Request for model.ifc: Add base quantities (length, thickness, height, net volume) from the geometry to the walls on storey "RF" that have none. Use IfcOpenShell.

First a look at what the model holds.

```python
import ifcopenshell
import ifcopenshell.util.element
import ifcopenshell.util.unit

model = ifcopenshell.open("model.ifc")
print(model.schema)
for unit_type in ("LENGTHUNIT", "AREAUNIT", "VOLUMEUNIT"):
    print(unit_type, ifcopenshell.util.unit.calculate_unit_scale(model, unit_type))
storey = next(s for s in model.by_type("IfcBuildingStorey") if s.Name == "RF")
walls = [e for e in ifcopenshell.util.element.get_decomposition(storey) if e.is_a("IfcWall")]
for e in sorted(walls, key=lambda e: e.id()):
    print(e.id(), e.is_a(), e.Name, list(ifcopenshell.util.element.get_psets(e, qtos_only=True)), sep=" | ")
```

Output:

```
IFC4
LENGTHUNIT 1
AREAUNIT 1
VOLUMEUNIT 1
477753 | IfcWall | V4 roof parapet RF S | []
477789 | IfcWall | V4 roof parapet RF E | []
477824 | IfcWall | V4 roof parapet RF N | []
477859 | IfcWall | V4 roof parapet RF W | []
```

```python
import ifcopenshell
import ifcopenshell.api.pset
import ifcopenshell.geom
import ifcopenshell.util.element
import ifcopenshell.util.shape
import ifcopenshell.util.unit

model = ifcopenshell.open("model.ifc")
unit_scale = ifcopenshell.util.unit.calculate_unit_scale(model)
volume_scale = ifcopenshell.util.unit.calculate_unit_scale(model, "VOLUMEUNIT")
settings = ifcopenshell.geom.settings()

storey = next(s for s in model.by_type("IfcBuildingStorey") if s.Name == "RF")
walls = [e for e in ifcopenshell.util.element.get_decomposition(storey) if e.is_a("IfcWall")]

for e in sorted(walls, key=lambda e: e.id()):
    if ifcopenshell.util.element.get_psets(e, qtos_only=True, should_inherit=False):
        continue
    # Geometry comes back in metres, in the element's own axes.
    shape = ifcopenshell.geom.create_shape(settings, e)
    values = {
        "Length": ifcopenshell.util.shape.get_x(shape.geometry) / unit_scale,
        "Width": ifcopenshell.util.shape.get_y(shape.geometry) / unit_scale,
        "Height": ifcopenshell.util.shape.get_z(shape.geometry) / unit_scale,
        "NetVolume": ifcopenshell.util.shape.get_volume(shape.geometry) / volume_scale,
    }
    qto = ifcopenshell.api.pset.add_qto(model, product=e, name="Qto_WallBaseQuantities")
    ifcopenshell.api.pset.edit_qto(model, qto=qto, properties=values)
    print(e.id(), {k: round(v, 3) for k, v in values.items()})

model.write("model-out.ifc")
```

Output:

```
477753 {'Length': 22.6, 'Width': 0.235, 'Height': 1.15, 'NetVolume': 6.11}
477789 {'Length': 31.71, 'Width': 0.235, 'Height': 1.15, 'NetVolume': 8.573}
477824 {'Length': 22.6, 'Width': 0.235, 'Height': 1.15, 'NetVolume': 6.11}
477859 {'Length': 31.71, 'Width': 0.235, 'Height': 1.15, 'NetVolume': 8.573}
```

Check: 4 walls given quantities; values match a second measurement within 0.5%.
